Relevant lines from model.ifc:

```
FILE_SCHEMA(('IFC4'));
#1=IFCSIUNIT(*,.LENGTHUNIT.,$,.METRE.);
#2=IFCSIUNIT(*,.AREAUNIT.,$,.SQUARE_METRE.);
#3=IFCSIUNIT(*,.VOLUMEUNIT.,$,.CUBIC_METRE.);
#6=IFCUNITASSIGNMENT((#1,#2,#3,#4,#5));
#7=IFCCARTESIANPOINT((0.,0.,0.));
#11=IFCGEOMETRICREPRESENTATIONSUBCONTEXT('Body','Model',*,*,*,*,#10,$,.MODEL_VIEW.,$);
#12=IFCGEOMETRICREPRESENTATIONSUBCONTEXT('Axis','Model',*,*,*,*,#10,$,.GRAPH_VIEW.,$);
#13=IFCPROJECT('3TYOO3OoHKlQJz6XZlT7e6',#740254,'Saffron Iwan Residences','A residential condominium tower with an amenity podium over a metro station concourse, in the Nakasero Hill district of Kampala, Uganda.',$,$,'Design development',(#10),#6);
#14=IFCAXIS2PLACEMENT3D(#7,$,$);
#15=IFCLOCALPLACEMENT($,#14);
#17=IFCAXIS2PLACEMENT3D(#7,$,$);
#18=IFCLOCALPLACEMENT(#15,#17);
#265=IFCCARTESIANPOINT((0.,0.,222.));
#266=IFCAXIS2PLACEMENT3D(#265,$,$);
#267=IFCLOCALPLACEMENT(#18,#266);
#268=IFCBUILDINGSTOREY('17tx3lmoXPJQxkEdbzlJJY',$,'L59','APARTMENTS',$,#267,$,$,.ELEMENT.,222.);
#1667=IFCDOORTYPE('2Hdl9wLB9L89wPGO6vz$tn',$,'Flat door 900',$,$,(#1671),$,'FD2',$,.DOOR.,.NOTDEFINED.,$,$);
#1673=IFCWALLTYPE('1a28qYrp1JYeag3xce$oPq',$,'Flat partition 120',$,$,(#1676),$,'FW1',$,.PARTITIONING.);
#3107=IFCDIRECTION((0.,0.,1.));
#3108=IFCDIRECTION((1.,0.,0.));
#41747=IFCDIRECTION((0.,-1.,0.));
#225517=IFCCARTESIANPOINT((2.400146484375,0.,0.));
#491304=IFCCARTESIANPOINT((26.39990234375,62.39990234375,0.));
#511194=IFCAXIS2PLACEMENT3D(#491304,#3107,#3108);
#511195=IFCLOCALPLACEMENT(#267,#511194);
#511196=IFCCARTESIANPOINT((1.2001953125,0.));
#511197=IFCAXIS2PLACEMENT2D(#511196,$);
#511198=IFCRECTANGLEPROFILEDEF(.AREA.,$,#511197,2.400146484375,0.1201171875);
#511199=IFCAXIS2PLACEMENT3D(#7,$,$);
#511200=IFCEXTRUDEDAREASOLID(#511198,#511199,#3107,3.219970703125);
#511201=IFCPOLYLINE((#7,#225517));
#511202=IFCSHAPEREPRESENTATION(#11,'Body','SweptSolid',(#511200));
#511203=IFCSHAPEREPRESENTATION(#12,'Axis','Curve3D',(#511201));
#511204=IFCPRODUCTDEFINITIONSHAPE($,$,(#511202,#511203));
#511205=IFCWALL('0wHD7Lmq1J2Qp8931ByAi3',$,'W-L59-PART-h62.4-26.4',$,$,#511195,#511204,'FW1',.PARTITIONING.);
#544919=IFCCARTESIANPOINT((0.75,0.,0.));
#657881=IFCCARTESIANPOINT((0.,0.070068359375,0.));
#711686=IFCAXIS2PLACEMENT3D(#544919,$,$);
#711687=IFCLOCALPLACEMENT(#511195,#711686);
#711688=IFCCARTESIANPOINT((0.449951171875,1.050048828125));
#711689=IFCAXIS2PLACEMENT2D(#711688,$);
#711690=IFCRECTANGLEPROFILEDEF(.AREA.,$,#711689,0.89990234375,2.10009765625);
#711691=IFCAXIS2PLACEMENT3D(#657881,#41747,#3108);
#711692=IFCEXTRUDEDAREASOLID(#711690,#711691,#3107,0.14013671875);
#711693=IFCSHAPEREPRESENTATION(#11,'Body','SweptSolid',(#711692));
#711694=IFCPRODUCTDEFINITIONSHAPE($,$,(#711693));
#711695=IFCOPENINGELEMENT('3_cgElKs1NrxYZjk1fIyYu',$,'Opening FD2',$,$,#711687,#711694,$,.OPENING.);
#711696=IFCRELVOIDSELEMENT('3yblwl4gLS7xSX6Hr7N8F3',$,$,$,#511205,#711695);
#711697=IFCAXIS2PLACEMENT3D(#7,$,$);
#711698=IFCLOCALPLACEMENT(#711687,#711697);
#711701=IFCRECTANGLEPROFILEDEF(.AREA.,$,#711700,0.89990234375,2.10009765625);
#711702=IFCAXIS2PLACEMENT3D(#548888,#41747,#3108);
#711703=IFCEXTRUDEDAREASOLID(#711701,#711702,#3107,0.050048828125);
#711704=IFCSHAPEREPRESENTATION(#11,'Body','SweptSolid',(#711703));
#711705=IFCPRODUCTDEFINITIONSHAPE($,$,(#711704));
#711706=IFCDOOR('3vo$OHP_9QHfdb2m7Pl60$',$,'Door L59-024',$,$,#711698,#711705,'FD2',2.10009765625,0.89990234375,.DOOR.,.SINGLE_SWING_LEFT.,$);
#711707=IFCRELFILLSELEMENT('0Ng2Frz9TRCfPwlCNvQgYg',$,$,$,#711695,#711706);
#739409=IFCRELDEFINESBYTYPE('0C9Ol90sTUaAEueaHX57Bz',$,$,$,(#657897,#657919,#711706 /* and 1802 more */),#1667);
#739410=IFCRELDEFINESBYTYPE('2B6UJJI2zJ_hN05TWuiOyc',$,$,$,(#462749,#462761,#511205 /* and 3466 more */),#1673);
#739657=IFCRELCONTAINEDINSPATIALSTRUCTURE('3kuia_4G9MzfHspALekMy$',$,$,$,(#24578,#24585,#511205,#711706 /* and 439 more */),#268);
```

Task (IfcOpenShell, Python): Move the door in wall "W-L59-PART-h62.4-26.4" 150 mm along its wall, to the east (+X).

```python
import ifcopenshell
import ifcopenshell.api.geometry
import ifcopenshell.util.placement
import ifcopenshell.util.unit

model = ifcopenshell.open("model.ifc")
unit_scale = ifcopenshell.util.unit.calculate_unit_scale(model)

door = model.by_id(711706)
opening = door.FillsVoids[0].RelatingOpeningElement
wall = opening.VoidsElements[0].RelatingBuildingElement

wall_matrix = ifcopenshell.util.placement.get_local_placement(wall.ObjectPlacement)
shift = wall_matrix[:3, 0] * 0.15 / unit_scale
before = ifcopenshell.util.placement.get_local_placement(door.ObjectPlacement)[:3, 3].copy()

# The door is placed relative to its opening, so it follows when the opening moves.
matrix = ifcopenshell.util.placement.get_local_placement(opening.ObjectPlacement)
matrix[:3, 3] += shift
ifcopenshell.api.geometry.edit_object_placement(
    model, product=opening, matrix=matrix, is_si=False, should_transform_children=True
)

after = ifcopenshell.util.placement.get_local_placement(door.ObjectPlacement)[:3, 3]
print("door moved by", (after - before).round(3) + 0.0)

model.write("model_updated.ifc")
```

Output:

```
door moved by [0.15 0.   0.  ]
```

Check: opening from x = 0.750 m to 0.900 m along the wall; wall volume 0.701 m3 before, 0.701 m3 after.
